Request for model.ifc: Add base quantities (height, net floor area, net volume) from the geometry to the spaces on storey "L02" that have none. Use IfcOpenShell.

First a look at what the model holds.

```python
import ifcopenshell
import ifcopenshell.util.element
import ifcopenshell.util.unit

model = ifcopenshell.open("model.ifc")
print(model.schema)
for unit_type in ("LENGTHUNIT", "AREAUNIT", "VOLUMEUNIT"):
    print(unit_type, ifcopenshell.util.unit.calculate_unit_scale(model, unit_type))
storey = next(s for s in model.by_type("IfcBuildingStorey") if s.Name == "L02")
spaces = [e for e in ifcopenshell.util.element.get_decomposition(storey) if e.is_a("IfcSpace")]
for e in sorted(spaces, key=lambda e: e.id()):
    print(e.id(), e.is_a(), e.Name, list(ifcopenshell.util.element.get_psets(e, qtos_only=True)), sep=" | ")
```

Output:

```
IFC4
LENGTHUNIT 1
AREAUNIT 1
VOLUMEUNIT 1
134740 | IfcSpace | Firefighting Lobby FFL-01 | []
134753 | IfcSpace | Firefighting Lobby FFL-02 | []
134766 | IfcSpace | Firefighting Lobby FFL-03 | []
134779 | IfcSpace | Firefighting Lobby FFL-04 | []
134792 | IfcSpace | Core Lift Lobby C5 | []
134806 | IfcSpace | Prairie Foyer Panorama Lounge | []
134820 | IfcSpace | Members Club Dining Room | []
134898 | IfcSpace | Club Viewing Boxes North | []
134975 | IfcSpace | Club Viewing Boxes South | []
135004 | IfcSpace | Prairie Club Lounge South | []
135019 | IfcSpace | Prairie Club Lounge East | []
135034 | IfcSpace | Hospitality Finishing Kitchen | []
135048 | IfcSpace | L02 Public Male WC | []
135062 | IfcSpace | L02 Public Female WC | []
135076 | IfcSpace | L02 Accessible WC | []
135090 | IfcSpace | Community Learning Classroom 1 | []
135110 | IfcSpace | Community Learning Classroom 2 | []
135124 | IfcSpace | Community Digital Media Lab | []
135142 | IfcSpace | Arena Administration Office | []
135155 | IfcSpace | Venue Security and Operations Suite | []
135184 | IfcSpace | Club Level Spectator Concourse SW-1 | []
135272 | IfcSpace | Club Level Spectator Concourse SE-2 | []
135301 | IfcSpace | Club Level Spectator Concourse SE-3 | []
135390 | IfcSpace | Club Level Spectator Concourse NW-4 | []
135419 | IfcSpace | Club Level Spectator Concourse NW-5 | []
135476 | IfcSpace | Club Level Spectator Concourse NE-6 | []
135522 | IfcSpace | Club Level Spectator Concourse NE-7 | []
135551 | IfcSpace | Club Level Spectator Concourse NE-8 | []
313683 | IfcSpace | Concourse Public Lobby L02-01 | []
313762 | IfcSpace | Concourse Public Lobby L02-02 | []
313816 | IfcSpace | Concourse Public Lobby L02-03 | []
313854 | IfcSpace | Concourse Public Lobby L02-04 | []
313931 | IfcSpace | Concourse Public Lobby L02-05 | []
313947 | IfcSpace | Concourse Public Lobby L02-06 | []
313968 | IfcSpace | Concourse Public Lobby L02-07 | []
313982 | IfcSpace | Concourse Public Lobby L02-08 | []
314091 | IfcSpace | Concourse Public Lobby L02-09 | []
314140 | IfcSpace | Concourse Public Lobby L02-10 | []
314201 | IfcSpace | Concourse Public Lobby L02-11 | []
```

```python
import ifcopenshell
import ifcopenshell.api.pset
import ifcopenshell.geom
import ifcopenshell.util.element
import ifcopenshell.util.shape
import ifcopenshell.util.unit

model = ifcopenshell.open("model.ifc")
unit_scale = ifcopenshell.util.unit.calculate_unit_scale(model)
area_scale = ifcopenshell.util.unit.calculate_unit_scale(model, "AREAUNIT")
volume_scale = ifcopenshell.util.unit.calculate_unit_scale(model, "VOLUMEUNIT")
settings = ifcopenshell.geom.settings()

storey = next(s for s in model.by_type("IfcBuildingStorey") if s.Name == "L02")
spaces = [e for e in ifcopenshell.util.element.get_decomposition(storey) if e.is_a("IfcSpace")]

for e in sorted(spaces, key=lambda e: e.id()):
    if ifcopenshell.util.element.get_psets(e, qtos_only=True, should_inherit=False):
        continue
    # Geometry comes back in metres, in the element's own axes.
    shape = ifcopenshell.geom.create_shape(settings, e)
    values = {
        "Height": ifcopenshell.util.shape.get_z(shape.geometry) / unit_scale,
        "NetFloorArea": ifcopenshell.util.shape.get_footprint_area(shape.geometry) / area_scale,
        "NetVolume": ifcopenshell.util.shape.get_volume(shape.geometry) / volume_scale,
    }
    qto = ifcopenshell.api.pset.add_qto(model, product=e, name="Qto_SpaceBaseQuantities")
    ifcopenshell.api.pset.edit_qto(model, qto=qto, properties=values)
    print(e.id(), {k: round(v, 3) for k, v in values.items()})

model.write("model_edited.ifc")
```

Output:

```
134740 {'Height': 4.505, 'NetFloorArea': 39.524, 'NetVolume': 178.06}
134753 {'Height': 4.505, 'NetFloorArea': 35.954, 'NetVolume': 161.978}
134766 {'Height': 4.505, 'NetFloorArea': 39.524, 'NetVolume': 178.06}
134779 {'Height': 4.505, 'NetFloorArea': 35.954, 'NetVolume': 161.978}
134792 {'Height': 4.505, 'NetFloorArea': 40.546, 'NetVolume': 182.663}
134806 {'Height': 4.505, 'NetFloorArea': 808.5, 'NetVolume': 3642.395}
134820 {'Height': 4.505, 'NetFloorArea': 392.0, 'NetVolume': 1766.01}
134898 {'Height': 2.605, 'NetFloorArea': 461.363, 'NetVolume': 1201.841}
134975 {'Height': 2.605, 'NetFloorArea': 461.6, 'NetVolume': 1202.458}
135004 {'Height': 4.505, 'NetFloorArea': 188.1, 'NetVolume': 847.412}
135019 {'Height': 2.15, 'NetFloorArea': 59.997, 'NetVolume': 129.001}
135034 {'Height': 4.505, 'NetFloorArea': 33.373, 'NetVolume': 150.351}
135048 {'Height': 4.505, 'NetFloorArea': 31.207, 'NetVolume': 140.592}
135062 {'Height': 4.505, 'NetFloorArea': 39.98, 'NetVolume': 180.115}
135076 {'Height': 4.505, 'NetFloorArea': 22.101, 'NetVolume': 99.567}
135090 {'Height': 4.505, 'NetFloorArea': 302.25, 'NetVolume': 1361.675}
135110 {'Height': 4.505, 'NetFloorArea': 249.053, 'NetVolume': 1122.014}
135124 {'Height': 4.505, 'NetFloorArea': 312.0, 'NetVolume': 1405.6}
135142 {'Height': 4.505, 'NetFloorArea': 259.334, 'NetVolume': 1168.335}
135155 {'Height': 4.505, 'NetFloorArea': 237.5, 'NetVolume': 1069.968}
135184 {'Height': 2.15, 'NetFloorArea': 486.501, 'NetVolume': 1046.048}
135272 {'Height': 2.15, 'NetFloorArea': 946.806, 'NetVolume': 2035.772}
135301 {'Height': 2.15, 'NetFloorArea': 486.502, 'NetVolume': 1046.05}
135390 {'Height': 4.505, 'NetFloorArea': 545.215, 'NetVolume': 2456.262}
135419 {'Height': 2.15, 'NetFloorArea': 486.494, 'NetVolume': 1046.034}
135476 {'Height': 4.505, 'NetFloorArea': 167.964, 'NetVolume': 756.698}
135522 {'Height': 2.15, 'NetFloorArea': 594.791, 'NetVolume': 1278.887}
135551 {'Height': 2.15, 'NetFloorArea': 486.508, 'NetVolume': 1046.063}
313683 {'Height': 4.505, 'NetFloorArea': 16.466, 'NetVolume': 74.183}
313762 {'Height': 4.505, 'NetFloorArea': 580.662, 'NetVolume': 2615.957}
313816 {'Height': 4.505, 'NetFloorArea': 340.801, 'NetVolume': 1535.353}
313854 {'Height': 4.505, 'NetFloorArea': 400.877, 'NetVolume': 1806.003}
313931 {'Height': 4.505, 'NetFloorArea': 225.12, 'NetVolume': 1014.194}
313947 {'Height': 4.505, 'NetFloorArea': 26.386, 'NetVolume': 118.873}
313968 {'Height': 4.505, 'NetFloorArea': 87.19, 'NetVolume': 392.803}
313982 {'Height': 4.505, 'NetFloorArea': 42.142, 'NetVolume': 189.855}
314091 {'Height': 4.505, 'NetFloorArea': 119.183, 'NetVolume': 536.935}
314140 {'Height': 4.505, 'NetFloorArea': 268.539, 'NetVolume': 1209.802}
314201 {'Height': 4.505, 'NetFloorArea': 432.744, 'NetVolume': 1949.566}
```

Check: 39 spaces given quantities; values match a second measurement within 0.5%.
